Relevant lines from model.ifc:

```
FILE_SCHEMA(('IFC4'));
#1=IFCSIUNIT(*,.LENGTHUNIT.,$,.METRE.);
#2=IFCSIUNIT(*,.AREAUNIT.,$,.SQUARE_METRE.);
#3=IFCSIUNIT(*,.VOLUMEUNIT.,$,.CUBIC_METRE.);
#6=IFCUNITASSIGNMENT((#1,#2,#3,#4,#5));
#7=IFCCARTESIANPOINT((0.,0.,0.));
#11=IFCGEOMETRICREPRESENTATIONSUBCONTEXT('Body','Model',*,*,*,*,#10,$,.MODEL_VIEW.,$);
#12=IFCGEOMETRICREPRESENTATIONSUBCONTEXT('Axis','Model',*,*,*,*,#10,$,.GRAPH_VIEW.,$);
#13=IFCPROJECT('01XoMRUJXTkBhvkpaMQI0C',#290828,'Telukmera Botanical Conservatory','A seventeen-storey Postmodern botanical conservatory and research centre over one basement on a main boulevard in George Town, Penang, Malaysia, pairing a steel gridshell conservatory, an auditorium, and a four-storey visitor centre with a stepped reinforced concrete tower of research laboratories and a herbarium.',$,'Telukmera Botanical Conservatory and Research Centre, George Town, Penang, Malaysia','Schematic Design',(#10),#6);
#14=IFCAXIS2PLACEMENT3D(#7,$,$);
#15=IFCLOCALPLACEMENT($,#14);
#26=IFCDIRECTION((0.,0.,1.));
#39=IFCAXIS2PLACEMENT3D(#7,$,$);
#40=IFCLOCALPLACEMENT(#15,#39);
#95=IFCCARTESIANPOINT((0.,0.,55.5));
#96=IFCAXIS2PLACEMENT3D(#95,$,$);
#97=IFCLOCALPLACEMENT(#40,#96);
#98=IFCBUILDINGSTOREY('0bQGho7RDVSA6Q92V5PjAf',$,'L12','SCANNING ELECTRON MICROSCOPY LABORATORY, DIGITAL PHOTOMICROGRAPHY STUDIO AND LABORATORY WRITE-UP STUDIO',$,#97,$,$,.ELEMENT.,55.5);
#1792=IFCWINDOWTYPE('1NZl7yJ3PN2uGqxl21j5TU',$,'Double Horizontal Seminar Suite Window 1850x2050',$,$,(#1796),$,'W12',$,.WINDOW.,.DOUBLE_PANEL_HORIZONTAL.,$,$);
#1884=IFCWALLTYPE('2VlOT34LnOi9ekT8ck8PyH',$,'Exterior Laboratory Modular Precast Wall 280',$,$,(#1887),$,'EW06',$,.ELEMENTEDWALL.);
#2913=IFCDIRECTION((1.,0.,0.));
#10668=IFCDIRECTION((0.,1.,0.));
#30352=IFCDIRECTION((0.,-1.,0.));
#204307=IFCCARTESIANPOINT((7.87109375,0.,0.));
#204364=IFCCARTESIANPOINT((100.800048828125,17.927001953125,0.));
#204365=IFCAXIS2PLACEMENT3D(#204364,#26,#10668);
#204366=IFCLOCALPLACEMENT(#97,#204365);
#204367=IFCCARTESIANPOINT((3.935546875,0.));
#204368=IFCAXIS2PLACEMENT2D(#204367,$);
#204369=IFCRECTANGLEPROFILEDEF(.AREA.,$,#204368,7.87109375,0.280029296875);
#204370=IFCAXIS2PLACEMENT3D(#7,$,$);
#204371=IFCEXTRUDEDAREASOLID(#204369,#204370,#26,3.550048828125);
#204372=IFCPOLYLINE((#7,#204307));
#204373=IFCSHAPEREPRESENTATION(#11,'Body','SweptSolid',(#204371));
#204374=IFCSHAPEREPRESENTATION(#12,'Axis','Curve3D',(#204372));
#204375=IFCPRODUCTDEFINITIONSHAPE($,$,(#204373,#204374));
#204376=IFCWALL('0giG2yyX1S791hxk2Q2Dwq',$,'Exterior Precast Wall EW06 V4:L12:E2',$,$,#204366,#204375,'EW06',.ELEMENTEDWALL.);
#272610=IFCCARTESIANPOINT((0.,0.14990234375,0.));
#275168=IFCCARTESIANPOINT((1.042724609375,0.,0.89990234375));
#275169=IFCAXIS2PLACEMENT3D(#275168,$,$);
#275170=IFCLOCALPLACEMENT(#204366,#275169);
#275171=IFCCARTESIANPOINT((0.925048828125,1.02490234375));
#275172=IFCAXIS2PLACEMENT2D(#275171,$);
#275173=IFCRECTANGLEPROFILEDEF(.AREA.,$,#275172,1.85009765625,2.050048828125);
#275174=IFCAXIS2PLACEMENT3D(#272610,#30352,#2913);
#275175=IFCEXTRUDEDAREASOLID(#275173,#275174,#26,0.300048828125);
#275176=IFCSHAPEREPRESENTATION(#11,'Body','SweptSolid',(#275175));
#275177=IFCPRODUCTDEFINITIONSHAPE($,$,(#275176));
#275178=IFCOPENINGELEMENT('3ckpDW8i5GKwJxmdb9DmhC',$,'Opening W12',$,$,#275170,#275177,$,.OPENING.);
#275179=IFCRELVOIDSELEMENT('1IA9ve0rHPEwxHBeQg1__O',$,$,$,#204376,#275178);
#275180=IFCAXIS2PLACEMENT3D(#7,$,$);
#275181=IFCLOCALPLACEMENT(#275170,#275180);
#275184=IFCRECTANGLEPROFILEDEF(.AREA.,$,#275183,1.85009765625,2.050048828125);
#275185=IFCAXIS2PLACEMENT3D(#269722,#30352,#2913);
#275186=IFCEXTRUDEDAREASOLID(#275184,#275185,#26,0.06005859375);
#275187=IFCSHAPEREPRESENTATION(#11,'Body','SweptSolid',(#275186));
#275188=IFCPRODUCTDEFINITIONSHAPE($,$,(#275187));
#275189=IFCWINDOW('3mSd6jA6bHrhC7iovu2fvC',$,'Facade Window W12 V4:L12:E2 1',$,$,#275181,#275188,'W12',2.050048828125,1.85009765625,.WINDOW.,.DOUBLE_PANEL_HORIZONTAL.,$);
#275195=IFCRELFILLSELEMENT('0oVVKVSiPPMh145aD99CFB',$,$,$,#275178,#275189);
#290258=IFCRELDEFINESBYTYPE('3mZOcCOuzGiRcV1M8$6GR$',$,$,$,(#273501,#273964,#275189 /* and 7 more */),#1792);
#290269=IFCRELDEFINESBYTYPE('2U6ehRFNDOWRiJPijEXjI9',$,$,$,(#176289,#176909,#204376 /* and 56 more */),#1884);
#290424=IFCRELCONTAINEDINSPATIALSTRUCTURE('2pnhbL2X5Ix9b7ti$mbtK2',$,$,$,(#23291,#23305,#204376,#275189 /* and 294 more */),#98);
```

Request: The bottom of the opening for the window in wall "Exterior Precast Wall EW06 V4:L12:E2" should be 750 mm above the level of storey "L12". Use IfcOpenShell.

```python
import numpy as np
import ifcopenshell
import ifcopenshell.api.geometry
import ifcopenshell.geom
import ifcopenshell.util.element
import ifcopenshell.util.placement
import ifcopenshell.util.shape
import ifcopenshell.util.unit

model = ifcopenshell.open("model.ifc")
unit_scale = ifcopenshell.util.unit.calculate_unit_scale(model)

window = model.by_guid("3mSd6jA6bHrhC7iovu2fvC")
opening = window.FillsVoids[0].RelatingOpeningElement
storey = ifcopenshell.util.element.get_container(window, ifc_class="IfcBuildingStorey")
level = ifcopenshell.util.placement.get_local_placement(storey.ObjectPlacement)[2, 3]

# The opening's origin need not be at the sill, so measure its lowest point.
shape = ifcopenshell.geom.create_shape(ifcopenshell.geom.settings(), opening)
bottom = ifcopenshell.util.shape.get_shape_bottom_elevation(shape, shape.geometry) / unit_scale
dz = level + 0.75 / unit_scale - bottom

shift = np.array([0.0, 0.0, dz])
# The window is placed relative to its opening, so it follows when the opening moves.
matrix = ifcopenshell.util.placement.get_local_placement(opening.ObjectPlacement)
matrix[:3, 3] += shift
ifcopenshell.api.geometry.edit_object_placement(
    model, product=opening, matrix=matrix, is_si=False, should_transform_children=True
)

print(f"moved by {dz * unit_scale:+.3f} m")

model.write("model_edited.ifc")
```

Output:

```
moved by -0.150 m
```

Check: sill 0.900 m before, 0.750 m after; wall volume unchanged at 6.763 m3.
